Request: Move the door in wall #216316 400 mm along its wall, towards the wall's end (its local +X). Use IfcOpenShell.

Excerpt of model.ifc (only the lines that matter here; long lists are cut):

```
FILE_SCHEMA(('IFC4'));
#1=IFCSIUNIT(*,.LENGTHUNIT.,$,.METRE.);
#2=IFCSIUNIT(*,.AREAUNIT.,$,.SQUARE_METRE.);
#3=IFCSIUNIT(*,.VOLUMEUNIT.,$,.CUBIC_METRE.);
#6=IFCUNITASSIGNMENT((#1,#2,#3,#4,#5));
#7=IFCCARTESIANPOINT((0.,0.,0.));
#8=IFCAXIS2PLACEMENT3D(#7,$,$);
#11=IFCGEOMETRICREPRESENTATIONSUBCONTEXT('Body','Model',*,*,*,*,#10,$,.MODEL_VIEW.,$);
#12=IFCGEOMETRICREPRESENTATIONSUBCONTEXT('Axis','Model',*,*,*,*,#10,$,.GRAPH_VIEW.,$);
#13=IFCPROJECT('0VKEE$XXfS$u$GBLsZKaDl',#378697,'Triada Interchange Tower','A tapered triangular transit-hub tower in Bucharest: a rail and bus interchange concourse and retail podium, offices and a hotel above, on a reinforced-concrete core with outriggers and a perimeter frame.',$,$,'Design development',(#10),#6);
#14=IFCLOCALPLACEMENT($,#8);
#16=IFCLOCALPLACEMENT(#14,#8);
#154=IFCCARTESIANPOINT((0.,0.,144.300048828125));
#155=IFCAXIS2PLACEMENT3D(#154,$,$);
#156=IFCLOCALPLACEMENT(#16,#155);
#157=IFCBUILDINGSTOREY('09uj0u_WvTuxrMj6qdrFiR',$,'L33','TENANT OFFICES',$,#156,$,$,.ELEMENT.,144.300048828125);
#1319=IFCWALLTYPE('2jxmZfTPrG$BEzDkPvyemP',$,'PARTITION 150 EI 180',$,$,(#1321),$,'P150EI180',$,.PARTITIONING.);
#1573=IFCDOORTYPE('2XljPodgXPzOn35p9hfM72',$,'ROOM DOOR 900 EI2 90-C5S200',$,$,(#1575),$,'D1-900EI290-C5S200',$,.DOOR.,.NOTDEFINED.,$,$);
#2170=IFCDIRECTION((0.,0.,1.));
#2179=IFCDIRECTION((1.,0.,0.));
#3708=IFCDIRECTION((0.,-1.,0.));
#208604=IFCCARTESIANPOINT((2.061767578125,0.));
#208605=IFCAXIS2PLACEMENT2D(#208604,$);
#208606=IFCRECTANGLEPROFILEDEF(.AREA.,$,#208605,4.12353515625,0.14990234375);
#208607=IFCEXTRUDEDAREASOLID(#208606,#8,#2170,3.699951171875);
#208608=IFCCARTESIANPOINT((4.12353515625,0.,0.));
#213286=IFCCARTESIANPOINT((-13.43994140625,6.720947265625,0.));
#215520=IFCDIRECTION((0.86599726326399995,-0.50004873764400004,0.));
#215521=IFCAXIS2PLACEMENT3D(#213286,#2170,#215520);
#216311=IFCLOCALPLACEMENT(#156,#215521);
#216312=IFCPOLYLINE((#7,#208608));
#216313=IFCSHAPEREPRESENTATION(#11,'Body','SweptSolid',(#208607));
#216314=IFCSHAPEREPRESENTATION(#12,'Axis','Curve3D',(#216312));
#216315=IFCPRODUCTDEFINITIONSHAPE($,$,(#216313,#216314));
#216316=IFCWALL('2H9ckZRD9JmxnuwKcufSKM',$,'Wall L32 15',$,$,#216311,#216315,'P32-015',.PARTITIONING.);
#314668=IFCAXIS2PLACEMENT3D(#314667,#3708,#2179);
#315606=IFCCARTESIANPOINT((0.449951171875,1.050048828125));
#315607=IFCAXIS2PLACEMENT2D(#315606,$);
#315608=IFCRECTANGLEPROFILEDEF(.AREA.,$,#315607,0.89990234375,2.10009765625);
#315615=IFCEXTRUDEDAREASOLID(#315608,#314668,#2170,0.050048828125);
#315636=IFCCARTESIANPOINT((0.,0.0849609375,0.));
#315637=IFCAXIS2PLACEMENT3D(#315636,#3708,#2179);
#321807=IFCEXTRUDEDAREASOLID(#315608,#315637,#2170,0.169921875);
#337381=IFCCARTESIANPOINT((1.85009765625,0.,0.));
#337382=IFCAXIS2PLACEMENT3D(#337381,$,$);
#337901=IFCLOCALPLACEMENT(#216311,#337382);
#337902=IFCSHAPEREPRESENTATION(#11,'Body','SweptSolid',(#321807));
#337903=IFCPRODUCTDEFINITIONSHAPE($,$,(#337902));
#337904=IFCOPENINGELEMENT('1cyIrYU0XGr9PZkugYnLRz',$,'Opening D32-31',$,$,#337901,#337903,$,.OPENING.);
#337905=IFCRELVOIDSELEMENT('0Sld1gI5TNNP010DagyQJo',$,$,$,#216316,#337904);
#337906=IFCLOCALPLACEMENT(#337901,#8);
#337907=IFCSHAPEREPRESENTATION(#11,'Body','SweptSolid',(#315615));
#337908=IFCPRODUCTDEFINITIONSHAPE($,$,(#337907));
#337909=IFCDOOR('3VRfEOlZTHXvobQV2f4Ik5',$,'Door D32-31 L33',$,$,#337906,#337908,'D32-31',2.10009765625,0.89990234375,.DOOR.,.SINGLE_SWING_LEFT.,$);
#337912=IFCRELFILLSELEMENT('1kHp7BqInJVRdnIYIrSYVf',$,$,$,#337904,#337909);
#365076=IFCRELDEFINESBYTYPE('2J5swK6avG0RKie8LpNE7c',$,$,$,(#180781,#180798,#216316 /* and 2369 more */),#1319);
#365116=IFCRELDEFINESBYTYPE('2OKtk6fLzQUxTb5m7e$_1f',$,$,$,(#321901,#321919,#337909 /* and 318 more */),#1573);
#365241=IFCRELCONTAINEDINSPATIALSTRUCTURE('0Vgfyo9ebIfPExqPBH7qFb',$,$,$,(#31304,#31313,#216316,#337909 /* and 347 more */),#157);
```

```python
import ifcopenshell
import ifcopenshell.api.geometry
import ifcopenshell.util.placement
import ifcopenshell.util.unit

model = ifcopenshell.open("model.ifc")
unit_scale = ifcopenshell.util.unit.calculate_unit_scale(model)

door = model.by_guid("3VRfEOlZTHXvobQV2f4Ik5")
opening = door.FillsVoids[0].RelatingOpeningElement
wall = opening.VoidsElements[0].RelatingBuildingElement

wall_matrix = ifcopenshell.util.placement.get_local_placement(wall.ObjectPlacement)
shift = wall_matrix[:3, 0] * 0.4 / unit_scale
before = ifcopenshell.util.placement.get_local_placement(door.ObjectPlacement)[:3, 3].copy()

# The door is placed relative to its opening, so it follows when the opening moves.
matrix = ifcopenshell.util.placement.get_local_placement(opening.ObjectPlacement)
matrix[:3, 3] += shift
ifcopenshell.api.geometry.edit_object_placement(
    model, product=opening, matrix=matrix, is_si=False, should_transform_children=True
)

after = ifcopenshell.util.placement.get_local_placement(door.ObjectPlacement)[:3, 3]
print("door moved by", (after - before).round(3) + 0.0)

model.write("model_updated.ifc")
```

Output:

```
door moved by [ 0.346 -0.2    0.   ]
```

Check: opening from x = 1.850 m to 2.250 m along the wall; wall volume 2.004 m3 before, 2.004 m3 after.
